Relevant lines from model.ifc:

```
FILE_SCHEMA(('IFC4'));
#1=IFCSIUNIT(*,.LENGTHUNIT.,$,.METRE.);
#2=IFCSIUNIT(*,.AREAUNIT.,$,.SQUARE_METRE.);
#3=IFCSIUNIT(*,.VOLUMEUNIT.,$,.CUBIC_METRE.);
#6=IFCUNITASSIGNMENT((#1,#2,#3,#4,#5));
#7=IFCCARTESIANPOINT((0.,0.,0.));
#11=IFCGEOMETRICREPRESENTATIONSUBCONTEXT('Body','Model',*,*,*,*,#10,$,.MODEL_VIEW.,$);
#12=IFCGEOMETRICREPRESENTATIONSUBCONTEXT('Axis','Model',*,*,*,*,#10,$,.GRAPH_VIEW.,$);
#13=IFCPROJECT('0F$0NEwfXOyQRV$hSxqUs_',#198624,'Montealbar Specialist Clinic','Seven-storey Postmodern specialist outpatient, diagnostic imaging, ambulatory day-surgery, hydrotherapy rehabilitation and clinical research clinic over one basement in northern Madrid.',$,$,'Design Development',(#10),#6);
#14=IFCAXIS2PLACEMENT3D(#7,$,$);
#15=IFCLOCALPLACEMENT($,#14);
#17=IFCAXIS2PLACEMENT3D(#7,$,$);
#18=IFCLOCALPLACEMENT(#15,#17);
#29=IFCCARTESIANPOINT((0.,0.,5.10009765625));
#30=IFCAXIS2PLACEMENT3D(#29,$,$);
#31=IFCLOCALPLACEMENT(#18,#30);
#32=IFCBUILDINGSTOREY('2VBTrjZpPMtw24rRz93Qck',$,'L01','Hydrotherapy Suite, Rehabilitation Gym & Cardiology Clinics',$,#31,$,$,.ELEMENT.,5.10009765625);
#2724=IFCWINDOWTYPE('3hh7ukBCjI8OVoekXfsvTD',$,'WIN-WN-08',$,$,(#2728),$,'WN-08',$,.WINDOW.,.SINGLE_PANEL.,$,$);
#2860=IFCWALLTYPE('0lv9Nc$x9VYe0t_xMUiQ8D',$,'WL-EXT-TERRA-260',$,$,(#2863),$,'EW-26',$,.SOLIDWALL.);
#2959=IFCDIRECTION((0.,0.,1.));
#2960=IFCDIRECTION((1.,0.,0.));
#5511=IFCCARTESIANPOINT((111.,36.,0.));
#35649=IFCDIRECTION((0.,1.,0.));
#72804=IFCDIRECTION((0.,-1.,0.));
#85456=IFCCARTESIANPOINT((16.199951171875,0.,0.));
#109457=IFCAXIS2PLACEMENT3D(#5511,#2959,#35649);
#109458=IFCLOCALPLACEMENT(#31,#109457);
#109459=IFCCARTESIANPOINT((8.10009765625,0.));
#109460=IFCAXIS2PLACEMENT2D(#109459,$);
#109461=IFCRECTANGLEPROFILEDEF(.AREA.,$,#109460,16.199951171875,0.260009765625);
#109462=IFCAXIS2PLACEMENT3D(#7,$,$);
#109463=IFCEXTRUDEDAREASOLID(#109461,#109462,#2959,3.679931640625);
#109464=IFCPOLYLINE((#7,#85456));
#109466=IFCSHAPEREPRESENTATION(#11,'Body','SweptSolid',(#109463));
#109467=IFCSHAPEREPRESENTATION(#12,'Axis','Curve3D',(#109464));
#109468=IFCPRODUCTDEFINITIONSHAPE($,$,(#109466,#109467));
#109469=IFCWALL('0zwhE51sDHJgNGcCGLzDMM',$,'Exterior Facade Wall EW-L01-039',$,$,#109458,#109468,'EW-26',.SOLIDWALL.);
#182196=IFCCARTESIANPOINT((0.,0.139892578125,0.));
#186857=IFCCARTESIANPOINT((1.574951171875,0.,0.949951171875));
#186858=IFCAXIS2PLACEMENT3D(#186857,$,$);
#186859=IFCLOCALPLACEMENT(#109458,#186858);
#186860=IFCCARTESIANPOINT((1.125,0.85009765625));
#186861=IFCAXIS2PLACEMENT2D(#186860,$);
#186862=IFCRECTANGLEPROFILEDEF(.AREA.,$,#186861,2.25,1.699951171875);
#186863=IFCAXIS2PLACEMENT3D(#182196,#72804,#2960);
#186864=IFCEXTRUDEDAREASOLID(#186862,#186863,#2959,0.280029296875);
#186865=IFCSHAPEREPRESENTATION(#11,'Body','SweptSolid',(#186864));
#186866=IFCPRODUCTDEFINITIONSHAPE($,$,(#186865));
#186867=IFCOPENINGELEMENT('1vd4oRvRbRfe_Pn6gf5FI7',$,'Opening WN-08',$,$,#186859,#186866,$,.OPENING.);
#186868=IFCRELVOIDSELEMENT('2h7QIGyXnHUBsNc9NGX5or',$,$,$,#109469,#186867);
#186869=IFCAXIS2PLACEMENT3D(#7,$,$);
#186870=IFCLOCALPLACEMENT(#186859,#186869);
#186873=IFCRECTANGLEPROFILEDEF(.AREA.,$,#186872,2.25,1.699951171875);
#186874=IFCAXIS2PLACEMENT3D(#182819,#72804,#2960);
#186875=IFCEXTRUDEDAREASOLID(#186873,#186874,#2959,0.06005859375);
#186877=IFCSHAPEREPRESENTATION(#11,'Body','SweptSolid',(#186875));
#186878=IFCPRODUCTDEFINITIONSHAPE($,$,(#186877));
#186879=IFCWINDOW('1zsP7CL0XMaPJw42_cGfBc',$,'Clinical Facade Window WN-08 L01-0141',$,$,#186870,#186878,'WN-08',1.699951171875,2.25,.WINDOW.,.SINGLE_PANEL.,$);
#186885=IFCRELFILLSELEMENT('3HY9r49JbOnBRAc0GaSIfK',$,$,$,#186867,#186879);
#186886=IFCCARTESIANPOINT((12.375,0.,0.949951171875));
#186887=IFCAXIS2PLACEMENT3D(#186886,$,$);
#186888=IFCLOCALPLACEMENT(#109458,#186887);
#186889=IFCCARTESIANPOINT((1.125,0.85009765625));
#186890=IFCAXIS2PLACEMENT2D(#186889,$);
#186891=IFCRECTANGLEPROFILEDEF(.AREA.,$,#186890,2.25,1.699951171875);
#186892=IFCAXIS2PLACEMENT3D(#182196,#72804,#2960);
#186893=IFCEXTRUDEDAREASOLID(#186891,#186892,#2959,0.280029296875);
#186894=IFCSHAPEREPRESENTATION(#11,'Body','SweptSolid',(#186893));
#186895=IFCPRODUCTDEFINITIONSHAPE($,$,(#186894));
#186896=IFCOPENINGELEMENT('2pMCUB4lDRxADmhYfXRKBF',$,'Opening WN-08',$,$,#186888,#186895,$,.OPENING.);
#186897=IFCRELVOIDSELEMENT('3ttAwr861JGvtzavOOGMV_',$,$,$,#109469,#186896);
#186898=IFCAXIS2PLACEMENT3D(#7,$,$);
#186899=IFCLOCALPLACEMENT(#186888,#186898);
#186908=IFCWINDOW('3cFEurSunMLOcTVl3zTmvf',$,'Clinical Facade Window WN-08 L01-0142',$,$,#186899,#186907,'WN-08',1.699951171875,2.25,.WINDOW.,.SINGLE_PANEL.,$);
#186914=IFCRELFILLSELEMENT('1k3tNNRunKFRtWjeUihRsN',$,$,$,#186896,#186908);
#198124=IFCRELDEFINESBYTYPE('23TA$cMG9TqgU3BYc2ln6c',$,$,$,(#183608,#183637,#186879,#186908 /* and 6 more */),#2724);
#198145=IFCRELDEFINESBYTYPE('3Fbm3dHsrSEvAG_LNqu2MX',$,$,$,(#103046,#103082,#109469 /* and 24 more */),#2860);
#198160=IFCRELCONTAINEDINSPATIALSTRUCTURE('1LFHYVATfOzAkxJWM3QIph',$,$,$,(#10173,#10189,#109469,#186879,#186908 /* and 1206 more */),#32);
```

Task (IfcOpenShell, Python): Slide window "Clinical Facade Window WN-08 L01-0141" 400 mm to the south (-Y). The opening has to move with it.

```python
import ifcopenshell
import ifcopenshell.api.geometry
import ifcopenshell.util.placement
import ifcopenshell.util.unit

model = ifcopenshell.open("model.ifc")
unit_scale = ifcopenshell.util.unit.calculate_unit_scale(model)

window = model.by_guid("1zsP7CL0XMaPJw42_cGfBc")
opening = window.FillsVoids[0].RelatingOpeningElement
wall = opening.VoidsElements[0].RelatingBuildingElement

wall_matrix = ifcopenshell.util.placement.get_local_placement(wall.ObjectPlacement)
shift = wall_matrix[:3, 0] * -0.4 / unit_scale
before = ifcopenshell.util.placement.get_local_placement(window.ObjectPlacement)[:3, 3].copy()

# The window is placed relative to its opening, so it follows when the opening moves.
matrix = ifcopenshell.util.placement.get_local_placement(opening.ObjectPlacement)
matrix[:3, 3] += shift
ifcopenshell.api.geometry.edit_object_placement(
    model, product=opening, matrix=matrix, is_si=False, should_transform_children=True
)

after = ifcopenshell.util.placement.get_local_placement(window.ObjectPlacement)[:3, 3]
print("window moved by", (after - before).round(3) + 0.0)

model.write("model_updated.ifc")
```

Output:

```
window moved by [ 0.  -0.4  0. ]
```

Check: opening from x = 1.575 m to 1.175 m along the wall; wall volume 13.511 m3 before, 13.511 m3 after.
